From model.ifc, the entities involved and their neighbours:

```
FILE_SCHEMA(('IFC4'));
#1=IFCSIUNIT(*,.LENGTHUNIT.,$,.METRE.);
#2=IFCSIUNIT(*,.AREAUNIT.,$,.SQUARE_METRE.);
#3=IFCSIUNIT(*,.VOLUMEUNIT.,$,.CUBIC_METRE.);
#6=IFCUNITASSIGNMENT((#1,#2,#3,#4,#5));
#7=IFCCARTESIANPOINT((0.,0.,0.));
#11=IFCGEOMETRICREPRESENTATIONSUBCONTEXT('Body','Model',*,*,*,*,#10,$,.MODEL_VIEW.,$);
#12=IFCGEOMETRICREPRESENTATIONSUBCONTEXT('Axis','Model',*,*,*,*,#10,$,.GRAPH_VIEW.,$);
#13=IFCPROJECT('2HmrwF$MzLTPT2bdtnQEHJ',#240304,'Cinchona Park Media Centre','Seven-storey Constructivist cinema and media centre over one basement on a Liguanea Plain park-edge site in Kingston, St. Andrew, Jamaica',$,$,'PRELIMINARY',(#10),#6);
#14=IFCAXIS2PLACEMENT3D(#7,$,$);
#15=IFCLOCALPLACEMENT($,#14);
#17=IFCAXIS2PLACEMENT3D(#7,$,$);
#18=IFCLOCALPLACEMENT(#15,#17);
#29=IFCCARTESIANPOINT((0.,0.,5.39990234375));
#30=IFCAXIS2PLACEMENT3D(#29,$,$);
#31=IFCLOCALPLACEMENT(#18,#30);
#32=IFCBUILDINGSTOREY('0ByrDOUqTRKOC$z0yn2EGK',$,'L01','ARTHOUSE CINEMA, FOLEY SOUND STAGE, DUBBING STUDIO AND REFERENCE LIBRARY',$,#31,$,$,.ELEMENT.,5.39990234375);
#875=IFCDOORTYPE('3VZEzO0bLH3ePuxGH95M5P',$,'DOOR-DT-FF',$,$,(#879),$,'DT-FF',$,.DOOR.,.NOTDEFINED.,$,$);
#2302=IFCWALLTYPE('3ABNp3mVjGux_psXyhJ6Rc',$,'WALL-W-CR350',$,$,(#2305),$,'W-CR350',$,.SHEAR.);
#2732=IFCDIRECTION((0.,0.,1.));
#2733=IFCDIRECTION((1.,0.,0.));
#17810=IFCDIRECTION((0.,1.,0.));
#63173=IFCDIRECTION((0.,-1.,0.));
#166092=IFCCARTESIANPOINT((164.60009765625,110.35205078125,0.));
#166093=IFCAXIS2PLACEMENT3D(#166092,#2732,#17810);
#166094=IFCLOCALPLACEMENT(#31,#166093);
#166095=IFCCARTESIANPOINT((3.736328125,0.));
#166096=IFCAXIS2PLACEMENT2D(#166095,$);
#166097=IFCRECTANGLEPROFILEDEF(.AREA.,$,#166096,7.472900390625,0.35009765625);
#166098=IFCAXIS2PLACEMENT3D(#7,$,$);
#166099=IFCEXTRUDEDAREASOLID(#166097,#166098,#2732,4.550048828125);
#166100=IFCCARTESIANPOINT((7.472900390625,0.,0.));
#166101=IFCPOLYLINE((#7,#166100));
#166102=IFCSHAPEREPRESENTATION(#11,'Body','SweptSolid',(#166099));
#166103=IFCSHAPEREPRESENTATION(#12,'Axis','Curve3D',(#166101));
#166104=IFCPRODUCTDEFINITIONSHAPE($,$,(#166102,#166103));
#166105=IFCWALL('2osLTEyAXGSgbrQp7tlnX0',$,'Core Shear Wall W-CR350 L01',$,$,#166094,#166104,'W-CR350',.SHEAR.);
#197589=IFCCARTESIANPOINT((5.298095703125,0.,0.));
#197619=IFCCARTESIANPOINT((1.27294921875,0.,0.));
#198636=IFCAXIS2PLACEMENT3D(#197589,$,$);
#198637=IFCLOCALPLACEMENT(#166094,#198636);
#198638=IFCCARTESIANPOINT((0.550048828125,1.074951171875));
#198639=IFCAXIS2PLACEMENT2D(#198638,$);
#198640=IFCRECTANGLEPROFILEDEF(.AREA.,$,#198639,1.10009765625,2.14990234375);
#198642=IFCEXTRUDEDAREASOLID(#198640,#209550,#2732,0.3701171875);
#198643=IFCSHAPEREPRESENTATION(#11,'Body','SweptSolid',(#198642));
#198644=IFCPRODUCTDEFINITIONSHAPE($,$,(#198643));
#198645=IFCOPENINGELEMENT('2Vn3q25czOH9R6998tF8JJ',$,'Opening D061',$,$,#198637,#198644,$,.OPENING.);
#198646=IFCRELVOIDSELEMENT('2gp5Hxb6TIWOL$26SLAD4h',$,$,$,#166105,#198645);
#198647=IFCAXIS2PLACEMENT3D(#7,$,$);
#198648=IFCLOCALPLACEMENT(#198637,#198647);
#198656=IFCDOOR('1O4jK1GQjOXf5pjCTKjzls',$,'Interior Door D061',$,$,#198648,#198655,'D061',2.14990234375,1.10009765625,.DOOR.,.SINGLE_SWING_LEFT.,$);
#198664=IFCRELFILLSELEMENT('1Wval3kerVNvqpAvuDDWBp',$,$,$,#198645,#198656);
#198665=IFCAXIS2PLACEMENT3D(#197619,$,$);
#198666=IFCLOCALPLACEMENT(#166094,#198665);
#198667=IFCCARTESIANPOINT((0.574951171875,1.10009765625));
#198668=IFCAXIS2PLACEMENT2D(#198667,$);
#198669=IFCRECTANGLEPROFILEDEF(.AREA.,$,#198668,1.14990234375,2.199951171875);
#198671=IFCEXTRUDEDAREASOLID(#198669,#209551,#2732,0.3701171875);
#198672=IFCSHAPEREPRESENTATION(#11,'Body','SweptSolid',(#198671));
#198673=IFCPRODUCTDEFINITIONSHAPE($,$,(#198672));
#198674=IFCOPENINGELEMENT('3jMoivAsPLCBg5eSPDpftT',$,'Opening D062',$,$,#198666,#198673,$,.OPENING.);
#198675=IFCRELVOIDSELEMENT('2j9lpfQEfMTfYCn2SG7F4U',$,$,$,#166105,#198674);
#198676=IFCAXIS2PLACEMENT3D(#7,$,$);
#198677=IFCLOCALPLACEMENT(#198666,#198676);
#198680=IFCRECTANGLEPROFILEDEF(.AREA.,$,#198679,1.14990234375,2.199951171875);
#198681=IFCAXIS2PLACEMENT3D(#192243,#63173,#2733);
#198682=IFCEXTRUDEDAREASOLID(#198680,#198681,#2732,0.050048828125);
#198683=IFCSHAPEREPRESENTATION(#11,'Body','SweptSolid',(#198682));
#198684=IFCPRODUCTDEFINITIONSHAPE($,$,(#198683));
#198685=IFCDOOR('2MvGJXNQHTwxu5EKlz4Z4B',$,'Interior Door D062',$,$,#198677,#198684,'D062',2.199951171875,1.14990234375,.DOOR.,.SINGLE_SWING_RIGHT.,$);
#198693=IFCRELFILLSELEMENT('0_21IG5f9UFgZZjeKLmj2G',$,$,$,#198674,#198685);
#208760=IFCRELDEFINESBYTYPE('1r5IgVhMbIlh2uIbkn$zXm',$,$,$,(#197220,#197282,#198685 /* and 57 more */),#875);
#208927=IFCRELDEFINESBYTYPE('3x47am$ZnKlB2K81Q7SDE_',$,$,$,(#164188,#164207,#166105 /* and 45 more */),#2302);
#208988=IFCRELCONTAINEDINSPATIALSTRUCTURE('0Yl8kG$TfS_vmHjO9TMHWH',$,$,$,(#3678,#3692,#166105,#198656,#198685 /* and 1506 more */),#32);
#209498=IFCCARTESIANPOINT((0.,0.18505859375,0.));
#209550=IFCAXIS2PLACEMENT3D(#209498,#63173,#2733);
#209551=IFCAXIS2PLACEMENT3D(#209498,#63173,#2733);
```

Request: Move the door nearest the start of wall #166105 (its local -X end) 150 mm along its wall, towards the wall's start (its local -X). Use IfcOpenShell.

```python
import ifcopenshell
import ifcopenshell.api.geometry
import ifcopenshell.util.placement

model = ifcopenshell.open("model.ifc")

door = model.by_guid("2MvGJXNQHTwxu5EKlz4Z4B")
opening = door.FillsVoids[0].RelatingOpeningElement
wall = opening.VoidsElements[0].RelatingBuildingElement

wall_matrix = ifcopenshell.util.placement.get_local_placement(wall.ObjectPlacement)
shift = wall_matrix[:3, 0] * -0.15
before = ifcopenshell.util.placement.get_local_placement(door.ObjectPlacement)[:3, 3].copy()

# The door is placed relative to its opening, so it follows when the opening moves.
matrix = ifcopenshell.util.placement.get_local_placement(opening.ObjectPlacement)
matrix[:3, 3] += shift
ifcopenshell.api.geometry.edit_object_placement(
    model, product=opening, matrix=matrix, is_si=False, should_transform_children=True
)

after = ifcopenshell.util.placement.get_local_placement(door.ObjectPlacement)[:3, 3]
print("door moved by", (after - before).round(3) + 0.0)

model.write("model_v2.ifc")
```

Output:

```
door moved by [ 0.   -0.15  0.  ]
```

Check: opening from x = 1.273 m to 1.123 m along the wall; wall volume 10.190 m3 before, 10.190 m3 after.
